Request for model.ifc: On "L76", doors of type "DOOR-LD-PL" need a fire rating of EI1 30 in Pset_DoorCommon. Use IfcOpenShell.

First a look at what the model holds.

```python
import ifcopenshell
import ifcopenshell.util.element

model = ifcopenshell.open("model.ifc")
print(model.schema)
storey = next(s for s in model.by_type("IfcBuildingStorey") if s.Name == "L76")
doors = [e for e in ifcopenshell.util.element.get_decomposition(storey) if e.is_a("IfcDoor")]
seen = {}
for e in doors:
    element_type = ifcopenshell.util.element.get_type(e)
    key = (element_type.Name if element_type != e and element_type else None, ifcopenshell.util.element.get_pset(e, "Pset_DoorCommon", "FireRating"))
    seen[key] = seen.get(key, 0) + 1
for (name, value), count in sorted(seen.items(), key=str):
    print(count, "x", name, "|", value)
```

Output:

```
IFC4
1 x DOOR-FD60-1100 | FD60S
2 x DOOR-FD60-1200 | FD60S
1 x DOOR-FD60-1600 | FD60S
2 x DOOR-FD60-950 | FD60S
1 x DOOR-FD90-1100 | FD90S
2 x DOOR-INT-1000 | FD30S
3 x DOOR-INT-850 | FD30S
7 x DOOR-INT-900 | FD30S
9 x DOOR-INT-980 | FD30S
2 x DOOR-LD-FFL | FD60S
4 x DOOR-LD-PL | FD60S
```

```python
import ifcopenshell
import ifcopenshell.api.pset
import ifcopenshell.util.element

model = ifcopenshell.open("model.ifc")

storey = next(s for s in model.by_type("IfcBuildingStorey") if s.Name == "L76")
doors = [e for e in ifcopenshell.util.element.get_decomposition(storey) if e.is_a("IfcDoor")]

count = 0
for e in doors:
    element_type = ifcopenshell.util.element.get_type(e)
    if element_type in (None, e) or element_type.Name != "DOOR-LD-PL":
        continue
    # add_pset returns the element's existing set when there is one.
    pset = ifcopenshell.api.pset.add_pset(model, product=e, name="Pset_DoorCommon")
    ifcopenshell.api.pset.edit_pset(model, pset=pset, properties={"FireRating": "EI1 30"})
    count += 1

print(count, "doors updated")

model.write("model_updated.ifc")
```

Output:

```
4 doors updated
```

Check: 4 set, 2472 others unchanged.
